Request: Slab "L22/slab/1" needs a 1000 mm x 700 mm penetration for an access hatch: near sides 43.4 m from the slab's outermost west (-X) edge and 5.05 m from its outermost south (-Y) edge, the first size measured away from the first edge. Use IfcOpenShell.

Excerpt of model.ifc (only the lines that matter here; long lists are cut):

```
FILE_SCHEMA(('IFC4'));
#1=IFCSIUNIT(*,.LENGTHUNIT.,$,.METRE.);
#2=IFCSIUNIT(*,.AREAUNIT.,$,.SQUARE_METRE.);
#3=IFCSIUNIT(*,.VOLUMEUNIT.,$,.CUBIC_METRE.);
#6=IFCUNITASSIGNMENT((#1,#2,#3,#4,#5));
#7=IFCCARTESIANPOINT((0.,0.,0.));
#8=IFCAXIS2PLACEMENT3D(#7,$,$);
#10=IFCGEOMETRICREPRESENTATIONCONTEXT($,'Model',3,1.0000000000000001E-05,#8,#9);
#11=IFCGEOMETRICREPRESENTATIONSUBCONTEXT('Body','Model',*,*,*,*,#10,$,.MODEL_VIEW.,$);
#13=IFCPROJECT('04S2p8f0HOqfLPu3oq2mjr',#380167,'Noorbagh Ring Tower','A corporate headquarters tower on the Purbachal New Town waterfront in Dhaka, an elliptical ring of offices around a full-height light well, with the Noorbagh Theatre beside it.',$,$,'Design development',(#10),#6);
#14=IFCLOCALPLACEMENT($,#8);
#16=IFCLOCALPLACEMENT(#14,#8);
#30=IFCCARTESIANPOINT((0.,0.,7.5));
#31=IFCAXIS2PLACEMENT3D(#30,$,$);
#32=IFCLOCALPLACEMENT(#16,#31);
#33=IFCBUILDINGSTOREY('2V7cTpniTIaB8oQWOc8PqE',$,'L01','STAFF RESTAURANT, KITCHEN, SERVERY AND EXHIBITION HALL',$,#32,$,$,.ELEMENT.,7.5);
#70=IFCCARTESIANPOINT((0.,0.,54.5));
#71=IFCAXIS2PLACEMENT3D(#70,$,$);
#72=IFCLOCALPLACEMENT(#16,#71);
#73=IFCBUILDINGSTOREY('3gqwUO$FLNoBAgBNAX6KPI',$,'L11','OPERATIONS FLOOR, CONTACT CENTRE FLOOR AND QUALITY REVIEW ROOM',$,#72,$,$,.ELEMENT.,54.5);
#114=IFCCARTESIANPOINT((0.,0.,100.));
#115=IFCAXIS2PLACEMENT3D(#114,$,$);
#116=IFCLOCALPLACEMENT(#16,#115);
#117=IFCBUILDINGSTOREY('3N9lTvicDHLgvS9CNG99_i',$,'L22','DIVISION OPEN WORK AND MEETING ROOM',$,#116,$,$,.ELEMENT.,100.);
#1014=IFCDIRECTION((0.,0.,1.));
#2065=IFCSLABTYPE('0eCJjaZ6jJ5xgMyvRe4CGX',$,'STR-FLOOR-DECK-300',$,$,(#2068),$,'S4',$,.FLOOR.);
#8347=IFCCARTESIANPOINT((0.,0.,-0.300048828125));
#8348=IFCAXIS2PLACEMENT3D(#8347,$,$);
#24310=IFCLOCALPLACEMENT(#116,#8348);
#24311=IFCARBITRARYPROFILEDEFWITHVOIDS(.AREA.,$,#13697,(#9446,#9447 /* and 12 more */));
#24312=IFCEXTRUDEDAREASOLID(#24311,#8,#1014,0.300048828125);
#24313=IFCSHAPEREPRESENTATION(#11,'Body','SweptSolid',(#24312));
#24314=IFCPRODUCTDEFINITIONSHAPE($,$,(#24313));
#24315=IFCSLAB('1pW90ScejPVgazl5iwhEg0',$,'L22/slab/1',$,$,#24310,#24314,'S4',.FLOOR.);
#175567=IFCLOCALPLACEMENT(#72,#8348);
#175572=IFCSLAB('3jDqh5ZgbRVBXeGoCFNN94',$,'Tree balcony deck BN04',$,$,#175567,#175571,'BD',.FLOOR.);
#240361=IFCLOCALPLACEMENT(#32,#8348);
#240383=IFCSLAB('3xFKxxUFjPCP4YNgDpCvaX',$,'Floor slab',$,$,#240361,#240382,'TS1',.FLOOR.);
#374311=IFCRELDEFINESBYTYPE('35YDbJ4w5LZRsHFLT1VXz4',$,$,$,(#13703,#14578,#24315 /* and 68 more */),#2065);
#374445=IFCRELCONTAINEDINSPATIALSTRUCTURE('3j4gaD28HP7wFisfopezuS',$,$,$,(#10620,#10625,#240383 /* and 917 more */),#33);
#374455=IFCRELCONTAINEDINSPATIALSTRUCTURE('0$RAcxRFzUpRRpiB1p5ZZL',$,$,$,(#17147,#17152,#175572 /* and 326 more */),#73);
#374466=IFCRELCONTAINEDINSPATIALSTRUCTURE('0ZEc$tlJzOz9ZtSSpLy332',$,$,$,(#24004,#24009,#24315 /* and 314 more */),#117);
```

```python
import numpy as np
import ifcopenshell
import ifcopenshell.api.feature
import ifcopenshell.api.geometry
import ifcopenshell.api.root
import ifcopenshell.geom
import ifcopenshell.util.placement
import ifcopenshell.util.representation
import ifcopenshell.util.shape
import ifcopenshell.util.unit

model = ifcopenshell.open("model.ifc")
unit_scale = ifcopenshell.util.unit.calculate_unit_scale(model)
settings = ifcopenshell.geom.settings()


def volume(element):
    """Net volume in cubic metres, openings subtracted."""
    shape = ifcopenshell.geom.create_shape(settings, element)
    return ifcopenshell.util.shape.get_volume(shape.geometry)


slab = model.by_id(24315)
before = volume(slab)

# Extent in the slab's own axes, in metres. The edges named are its -X and -Y sides.
slab_shape = ifcopenshell.geom.create_shape(settings, slab)
vertices = ifcopenshell.util.shape.get_vertices(slab_shape.geometry)
x_min, y_min, bottom = vertices.min(axis=0)
top = vertices[:, 2].max()

opening = ifcopenshell.api.root.create_entity(model, ifc_class="IfcOpeningElement", name="Access hatch opening", predefined_type="OPENING")
context = ifcopenshell.util.representation.get_context(model, "Model", "Body", "MODEL_VIEW")
width, depth = 1, 0.7
outline = [(0.0, 0.0), (width, 0.0), (width, depth), (0.0, depth), (0.0, 0.0)]
# Overshoot both faces by 50 mm so the cut is clean.
shape = ifcopenshell.api.geometry.add_slab_representation(
    model, context=context, depth=top - bottom + 0.1, polyline=outline
)
ifcopenshell.api.geometry.assign_representation(model, product=opening, representation=shape)

matrix = ifcopenshell.util.placement.get_local_placement(slab.ObjectPlacement)
matrix[:, 3] = matrix @ np.append(np.array([x_min + 43.4, y_min + 5.05, bottom - 0.05]) / unit_scale, 1.0)
ifcopenshell.api.geometry.edit_object_placement(model, product=opening, matrix=matrix, is_si=False)
ifcopenshell.api.feature.add_feature(model, feature=opening, element=slab)

after = volume(slab)

print(f"slab volume {before:.3f} -> {after:.3f} m3")

model.write("model_v2.ifc")
```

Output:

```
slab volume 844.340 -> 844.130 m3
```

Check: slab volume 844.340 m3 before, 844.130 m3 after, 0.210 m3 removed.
